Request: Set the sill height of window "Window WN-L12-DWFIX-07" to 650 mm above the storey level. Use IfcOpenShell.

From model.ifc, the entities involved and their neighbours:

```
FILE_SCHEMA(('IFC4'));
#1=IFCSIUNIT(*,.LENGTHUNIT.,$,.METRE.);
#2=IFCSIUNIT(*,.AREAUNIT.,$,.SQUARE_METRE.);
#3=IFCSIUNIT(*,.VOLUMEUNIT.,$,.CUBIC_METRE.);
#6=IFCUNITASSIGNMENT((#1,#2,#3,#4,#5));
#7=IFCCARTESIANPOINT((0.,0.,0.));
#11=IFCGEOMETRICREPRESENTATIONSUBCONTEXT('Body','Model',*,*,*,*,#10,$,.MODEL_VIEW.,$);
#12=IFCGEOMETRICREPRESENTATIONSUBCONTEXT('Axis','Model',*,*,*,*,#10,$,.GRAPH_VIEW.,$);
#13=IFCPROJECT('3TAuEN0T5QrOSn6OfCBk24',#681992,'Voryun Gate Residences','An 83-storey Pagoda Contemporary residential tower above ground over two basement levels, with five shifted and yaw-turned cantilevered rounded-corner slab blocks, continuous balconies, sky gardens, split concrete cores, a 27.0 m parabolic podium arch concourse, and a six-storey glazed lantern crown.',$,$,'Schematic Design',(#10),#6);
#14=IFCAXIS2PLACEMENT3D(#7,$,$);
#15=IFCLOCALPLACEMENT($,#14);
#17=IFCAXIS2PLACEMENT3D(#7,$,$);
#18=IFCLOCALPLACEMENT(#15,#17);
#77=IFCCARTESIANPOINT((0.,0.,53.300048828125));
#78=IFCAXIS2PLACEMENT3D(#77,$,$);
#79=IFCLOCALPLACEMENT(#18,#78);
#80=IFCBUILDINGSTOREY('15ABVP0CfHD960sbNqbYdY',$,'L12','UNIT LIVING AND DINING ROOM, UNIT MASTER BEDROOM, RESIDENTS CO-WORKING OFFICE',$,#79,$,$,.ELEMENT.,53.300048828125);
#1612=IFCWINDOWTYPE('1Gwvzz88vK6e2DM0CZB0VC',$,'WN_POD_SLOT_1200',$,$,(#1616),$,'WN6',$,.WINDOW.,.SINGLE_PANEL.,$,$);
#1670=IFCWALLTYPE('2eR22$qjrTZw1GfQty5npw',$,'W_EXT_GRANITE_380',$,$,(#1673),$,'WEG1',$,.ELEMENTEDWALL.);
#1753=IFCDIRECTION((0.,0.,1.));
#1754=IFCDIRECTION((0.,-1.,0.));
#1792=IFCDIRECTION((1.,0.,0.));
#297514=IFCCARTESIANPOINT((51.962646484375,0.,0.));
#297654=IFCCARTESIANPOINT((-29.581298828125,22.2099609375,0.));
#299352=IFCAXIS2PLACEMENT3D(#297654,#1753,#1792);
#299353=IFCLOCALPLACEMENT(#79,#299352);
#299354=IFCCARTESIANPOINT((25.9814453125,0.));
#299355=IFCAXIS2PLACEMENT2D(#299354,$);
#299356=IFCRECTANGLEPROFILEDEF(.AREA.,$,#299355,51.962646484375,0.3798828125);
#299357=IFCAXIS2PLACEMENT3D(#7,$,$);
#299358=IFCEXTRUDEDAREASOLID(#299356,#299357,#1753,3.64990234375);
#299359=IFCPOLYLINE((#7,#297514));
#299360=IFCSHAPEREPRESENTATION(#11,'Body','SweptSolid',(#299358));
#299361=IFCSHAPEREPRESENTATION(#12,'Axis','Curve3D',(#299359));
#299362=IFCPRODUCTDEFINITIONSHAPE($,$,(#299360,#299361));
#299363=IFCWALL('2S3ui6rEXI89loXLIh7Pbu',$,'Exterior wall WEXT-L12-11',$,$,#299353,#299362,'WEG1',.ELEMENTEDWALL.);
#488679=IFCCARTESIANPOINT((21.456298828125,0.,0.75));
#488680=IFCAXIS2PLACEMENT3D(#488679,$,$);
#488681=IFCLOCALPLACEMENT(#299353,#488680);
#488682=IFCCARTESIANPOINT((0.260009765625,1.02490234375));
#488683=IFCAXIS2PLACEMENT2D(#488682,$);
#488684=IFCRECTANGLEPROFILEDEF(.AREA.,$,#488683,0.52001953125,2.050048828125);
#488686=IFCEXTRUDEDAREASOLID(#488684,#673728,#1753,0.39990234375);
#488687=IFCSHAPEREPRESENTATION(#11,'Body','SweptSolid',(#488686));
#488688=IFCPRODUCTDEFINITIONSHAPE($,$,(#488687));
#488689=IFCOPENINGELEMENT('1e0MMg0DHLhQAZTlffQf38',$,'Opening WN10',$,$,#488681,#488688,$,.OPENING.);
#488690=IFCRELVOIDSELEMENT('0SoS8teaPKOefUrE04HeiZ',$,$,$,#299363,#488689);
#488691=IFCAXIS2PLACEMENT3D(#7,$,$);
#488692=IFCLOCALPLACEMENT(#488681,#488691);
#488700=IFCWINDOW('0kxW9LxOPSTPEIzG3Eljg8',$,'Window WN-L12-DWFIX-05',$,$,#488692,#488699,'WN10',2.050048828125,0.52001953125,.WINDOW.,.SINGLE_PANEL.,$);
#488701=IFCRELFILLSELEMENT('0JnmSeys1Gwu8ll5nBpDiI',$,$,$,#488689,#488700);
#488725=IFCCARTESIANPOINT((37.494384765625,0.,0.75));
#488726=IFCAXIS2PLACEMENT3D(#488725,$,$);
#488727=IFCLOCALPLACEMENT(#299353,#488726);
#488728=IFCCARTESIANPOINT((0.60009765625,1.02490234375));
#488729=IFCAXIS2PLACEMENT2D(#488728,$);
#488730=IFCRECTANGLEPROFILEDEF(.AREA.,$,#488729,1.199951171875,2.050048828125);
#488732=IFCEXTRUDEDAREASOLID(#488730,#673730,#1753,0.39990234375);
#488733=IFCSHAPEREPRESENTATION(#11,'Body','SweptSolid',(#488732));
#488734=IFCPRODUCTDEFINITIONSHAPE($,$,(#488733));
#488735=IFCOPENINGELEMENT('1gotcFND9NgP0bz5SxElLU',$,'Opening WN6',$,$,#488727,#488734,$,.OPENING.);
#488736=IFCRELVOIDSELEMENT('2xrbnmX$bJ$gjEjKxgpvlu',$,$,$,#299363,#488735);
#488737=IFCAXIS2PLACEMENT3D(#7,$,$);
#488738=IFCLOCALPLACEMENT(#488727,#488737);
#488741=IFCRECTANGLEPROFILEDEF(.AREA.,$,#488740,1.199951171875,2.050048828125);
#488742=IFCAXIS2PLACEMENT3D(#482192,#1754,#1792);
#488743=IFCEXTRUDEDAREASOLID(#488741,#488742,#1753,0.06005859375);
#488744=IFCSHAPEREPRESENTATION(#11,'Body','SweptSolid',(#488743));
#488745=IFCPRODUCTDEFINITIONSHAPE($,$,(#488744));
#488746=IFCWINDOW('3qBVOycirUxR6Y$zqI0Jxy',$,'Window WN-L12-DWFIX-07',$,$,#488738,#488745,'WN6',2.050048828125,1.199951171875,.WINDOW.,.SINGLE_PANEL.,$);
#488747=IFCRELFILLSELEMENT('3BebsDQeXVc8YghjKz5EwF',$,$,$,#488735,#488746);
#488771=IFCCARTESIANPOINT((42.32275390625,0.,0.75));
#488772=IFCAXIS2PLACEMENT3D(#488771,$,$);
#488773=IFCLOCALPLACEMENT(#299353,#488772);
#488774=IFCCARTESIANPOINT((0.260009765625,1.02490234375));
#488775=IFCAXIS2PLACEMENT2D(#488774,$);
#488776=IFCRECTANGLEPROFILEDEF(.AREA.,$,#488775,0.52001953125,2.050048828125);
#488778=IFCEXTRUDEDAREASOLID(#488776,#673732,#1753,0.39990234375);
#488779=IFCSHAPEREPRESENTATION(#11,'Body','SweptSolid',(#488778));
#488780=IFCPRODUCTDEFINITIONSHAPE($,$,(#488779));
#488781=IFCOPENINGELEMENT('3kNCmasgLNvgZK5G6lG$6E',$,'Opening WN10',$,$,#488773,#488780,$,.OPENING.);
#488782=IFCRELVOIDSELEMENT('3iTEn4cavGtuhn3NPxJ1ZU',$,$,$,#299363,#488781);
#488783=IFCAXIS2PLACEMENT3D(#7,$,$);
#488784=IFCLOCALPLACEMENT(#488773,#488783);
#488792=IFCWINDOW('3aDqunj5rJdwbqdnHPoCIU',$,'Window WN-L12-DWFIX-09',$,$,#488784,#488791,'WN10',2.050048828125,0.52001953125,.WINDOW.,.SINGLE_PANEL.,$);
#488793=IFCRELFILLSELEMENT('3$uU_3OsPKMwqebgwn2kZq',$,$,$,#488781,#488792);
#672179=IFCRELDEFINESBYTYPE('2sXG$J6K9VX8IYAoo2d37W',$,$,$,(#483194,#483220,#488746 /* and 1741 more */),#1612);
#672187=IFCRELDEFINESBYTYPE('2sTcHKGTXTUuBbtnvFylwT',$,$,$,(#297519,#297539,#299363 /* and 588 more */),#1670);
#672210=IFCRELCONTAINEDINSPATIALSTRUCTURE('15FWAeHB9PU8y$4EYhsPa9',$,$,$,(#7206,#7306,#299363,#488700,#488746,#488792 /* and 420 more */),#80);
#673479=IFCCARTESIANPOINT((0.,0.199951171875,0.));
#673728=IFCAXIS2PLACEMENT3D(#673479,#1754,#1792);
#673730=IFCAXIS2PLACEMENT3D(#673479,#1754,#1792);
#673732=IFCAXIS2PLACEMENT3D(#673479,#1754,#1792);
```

```python
import numpy as np
import ifcopenshell
import ifcopenshell.api.geometry
import ifcopenshell.geom
import ifcopenshell.util.element
import ifcopenshell.util.placement
import ifcopenshell.util.shape
import ifcopenshell.util.unit

model = ifcopenshell.open("model.ifc")
unit_scale = ifcopenshell.util.unit.calculate_unit_scale(model)

window = model.by_id(488746)
opening = window.FillsVoids[0].RelatingOpeningElement
storey = ifcopenshell.util.element.get_container(window, ifc_class="IfcBuildingStorey")
level = ifcopenshell.util.placement.get_local_placement(storey.ObjectPlacement)[2, 3]

# The opening's origin need not be at the sill, so measure its lowest point.
shape = ifcopenshell.geom.create_shape(ifcopenshell.geom.settings(), opening)
bottom = ifcopenshell.util.shape.get_shape_bottom_elevation(shape, shape.geometry) / unit_scale
dz = level + 0.65 / unit_scale - bottom

shift = np.array([0.0, 0.0, dz])
# The window is placed relative to its opening, so it follows when the opening moves.
matrix = ifcopenshell.util.placement.get_local_placement(opening.ObjectPlacement)
matrix[:3, 3] += shift
ifcopenshell.api.geometry.edit_object_placement(
    model, product=opening, matrix=matrix, is_si=False, should_transform_children=True
)

print(f"moved by {dz * unit_scale:+.3f} m")

model.write("model_updated.ifc")
```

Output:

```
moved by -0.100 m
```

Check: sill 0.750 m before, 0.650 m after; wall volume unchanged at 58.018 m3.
